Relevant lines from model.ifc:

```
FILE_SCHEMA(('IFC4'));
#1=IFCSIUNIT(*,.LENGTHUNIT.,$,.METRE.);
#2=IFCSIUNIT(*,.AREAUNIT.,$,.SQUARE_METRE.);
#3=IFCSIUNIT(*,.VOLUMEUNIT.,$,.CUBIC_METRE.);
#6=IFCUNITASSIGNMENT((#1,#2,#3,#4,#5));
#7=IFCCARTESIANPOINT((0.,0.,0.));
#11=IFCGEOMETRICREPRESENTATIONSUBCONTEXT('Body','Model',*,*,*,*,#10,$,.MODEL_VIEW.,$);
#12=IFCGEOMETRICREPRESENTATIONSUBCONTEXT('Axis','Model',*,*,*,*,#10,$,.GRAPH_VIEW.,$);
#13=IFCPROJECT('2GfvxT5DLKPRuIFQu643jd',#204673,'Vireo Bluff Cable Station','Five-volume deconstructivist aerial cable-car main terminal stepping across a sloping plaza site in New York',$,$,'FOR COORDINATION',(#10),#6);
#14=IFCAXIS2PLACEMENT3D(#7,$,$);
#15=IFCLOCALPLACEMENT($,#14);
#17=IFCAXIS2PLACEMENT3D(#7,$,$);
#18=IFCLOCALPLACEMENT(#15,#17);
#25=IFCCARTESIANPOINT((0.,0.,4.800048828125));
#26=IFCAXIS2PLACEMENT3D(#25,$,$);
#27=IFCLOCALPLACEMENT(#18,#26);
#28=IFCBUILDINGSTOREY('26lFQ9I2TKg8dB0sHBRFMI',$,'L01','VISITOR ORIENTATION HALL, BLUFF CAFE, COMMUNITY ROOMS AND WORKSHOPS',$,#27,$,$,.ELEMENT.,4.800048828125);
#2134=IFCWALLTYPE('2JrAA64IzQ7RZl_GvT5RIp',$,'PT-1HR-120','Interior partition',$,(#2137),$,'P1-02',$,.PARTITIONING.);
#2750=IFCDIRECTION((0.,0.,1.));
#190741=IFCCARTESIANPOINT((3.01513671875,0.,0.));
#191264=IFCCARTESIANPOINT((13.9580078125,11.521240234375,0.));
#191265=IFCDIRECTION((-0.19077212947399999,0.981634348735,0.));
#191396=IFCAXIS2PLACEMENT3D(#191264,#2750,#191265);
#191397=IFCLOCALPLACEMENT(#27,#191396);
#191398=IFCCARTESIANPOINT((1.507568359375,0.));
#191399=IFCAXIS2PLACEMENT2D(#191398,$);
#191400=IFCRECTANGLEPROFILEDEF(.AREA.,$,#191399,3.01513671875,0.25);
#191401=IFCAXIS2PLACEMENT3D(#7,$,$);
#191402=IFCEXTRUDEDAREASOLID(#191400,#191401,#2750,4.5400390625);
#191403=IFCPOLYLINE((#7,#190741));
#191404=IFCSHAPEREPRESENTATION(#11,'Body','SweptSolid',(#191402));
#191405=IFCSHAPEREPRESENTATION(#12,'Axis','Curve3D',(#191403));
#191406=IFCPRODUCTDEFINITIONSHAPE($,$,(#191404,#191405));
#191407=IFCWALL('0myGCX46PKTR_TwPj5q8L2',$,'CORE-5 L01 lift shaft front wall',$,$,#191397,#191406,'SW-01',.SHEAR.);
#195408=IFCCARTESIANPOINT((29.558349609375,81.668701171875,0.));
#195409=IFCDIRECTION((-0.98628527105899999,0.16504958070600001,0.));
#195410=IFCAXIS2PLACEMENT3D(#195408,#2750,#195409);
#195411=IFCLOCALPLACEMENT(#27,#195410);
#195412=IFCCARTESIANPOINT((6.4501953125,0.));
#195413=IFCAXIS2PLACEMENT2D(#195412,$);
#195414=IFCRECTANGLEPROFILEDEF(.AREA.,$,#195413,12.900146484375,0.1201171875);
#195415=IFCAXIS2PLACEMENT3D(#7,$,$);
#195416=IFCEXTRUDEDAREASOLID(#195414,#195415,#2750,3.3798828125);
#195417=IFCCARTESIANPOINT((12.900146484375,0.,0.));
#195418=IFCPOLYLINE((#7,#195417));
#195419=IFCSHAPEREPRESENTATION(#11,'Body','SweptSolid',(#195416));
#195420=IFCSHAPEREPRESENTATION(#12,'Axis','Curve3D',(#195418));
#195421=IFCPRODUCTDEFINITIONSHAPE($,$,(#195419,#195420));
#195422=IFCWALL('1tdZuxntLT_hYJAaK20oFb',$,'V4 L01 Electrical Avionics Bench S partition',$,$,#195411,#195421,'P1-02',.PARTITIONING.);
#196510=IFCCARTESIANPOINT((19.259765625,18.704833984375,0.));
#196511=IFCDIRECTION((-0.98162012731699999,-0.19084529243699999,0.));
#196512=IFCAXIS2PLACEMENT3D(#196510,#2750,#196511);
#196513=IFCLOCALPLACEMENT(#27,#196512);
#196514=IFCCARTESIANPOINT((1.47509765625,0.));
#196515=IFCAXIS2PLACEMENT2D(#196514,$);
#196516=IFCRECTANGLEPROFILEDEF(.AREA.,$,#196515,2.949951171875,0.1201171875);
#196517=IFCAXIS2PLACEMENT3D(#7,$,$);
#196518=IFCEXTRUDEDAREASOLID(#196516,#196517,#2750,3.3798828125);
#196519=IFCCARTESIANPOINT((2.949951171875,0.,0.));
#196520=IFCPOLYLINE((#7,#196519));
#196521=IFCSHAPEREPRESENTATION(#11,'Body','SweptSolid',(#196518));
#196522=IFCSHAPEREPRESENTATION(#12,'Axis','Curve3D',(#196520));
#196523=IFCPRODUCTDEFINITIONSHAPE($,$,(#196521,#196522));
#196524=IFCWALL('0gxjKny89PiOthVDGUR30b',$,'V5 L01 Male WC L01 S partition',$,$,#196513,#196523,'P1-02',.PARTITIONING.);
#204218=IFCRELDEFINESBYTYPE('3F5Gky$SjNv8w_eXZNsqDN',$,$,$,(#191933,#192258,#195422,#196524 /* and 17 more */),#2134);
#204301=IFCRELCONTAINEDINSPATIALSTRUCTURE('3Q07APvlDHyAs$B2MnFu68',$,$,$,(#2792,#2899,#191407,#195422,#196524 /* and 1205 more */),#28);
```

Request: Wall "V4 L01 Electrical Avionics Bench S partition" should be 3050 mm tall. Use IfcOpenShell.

```python
import ifcopenshell
import ifcopenshell.geom
import ifcopenshell.util.representation
import ifcopenshell.util.shape

model = ifcopenshell.open("model.ifc")
settings = ifcopenshell.geom.settings()


def volume(element):
    """Net volume in cubic metres, openings subtracted."""
    shape = ifcopenshell.geom.create_shape(settings, element)
    return ifcopenshell.util.shape.get_volume(shape.geometry)


wall = model.by_guid("1tdZuxntLT_hYJAaK20oFb")
before = volume(wall)

body = ifcopenshell.util.representation.get_representation(wall, "Model", "Body")
solid = body.Items[0]
old_height = solid.Depth
solid.Depth = 3.05
after = volume(wall)

print(f"height {old_height:g} -> {solid.Depth:g}, volume {before:.3f} -> {after:.3f} m3")

model.write("model_edited.ifc")
```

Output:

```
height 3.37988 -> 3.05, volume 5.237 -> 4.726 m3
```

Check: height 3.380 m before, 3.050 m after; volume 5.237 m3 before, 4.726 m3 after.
